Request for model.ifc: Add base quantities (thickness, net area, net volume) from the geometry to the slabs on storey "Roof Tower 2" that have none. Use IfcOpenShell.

First a look at what the model holds.

```python
import ifcopenshell
import ifcopenshell.util.element
import ifcopenshell.util.unit

model = ifcopenshell.open("model.ifc")
print(model.schema)
for unit_type in ("LENGTHUNIT", "AREAUNIT", "VOLUMEUNIT"):
    print(unit_type, ifcopenshell.util.unit.calculate_unit_scale(model, unit_type))
storey = next(s for s in model.by_type("IfcBuildingStorey") if s.Name == "Roof Tower 2")
slabs = [e for e in ifcopenshell.util.element.get_decomposition(storey) if e.is_a("IfcSlab")]
for e in sorted(slabs, key=lambda e: e.id()):
    print(e.id(), e.is_a(), e.Name, list(ifcopenshell.util.element.get_psets(e, qtos_only=True)), sep=" | ")
```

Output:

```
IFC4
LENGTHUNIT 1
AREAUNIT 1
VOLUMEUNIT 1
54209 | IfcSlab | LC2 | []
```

```python
import ifcopenshell
import ifcopenshell.api.pset
import ifcopenshell.geom
import ifcopenshell.util.element
import ifcopenshell.util.shape
import ifcopenshell.util.unit

model = ifcopenshell.open("model.ifc")
unit_scale = ifcopenshell.util.unit.calculate_unit_scale(model)
area_scale = ifcopenshell.util.unit.calculate_unit_scale(model, "AREAUNIT")
volume_scale = ifcopenshell.util.unit.calculate_unit_scale(model, "VOLUMEUNIT")
settings = ifcopenshell.geom.settings()

storey = next(s for s in model.by_type("IfcBuildingStorey") if s.Name == "Roof Tower 2")
slabs = [e for e in ifcopenshell.util.element.get_decomposition(storey) if e.is_a("IfcSlab")]

for e in sorted(slabs, key=lambda e: e.id()):
    if ifcopenshell.util.element.get_psets(e, qtos_only=True, should_inherit=False):
        continue
    # Geometry comes back in metres, in the element's own axes.
    shape = ifcopenshell.geom.create_shape(settings, e)
    values = {
        "Width": ifcopenshell.util.shape.get_z(shape.geometry) / unit_scale,
        "NetArea": ifcopenshell.util.shape.get_footprint_area(shape.geometry) / area_scale,
        "NetVolume": ifcopenshell.util.shape.get_volume(shape.geometry) / volume_scale,
    }
    qto = ifcopenshell.api.pset.add_qto(model, product=e, name="Qto_SlabBaseQuantities")
    ifcopenshell.api.pset.edit_qto(model, qto=qto, properties=values)
    print(e.id(), {k: round(v, 3) for k, v in values.items()})

model.write("model_v2.ifc")
```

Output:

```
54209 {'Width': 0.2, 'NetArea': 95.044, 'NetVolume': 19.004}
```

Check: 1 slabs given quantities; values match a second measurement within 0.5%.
